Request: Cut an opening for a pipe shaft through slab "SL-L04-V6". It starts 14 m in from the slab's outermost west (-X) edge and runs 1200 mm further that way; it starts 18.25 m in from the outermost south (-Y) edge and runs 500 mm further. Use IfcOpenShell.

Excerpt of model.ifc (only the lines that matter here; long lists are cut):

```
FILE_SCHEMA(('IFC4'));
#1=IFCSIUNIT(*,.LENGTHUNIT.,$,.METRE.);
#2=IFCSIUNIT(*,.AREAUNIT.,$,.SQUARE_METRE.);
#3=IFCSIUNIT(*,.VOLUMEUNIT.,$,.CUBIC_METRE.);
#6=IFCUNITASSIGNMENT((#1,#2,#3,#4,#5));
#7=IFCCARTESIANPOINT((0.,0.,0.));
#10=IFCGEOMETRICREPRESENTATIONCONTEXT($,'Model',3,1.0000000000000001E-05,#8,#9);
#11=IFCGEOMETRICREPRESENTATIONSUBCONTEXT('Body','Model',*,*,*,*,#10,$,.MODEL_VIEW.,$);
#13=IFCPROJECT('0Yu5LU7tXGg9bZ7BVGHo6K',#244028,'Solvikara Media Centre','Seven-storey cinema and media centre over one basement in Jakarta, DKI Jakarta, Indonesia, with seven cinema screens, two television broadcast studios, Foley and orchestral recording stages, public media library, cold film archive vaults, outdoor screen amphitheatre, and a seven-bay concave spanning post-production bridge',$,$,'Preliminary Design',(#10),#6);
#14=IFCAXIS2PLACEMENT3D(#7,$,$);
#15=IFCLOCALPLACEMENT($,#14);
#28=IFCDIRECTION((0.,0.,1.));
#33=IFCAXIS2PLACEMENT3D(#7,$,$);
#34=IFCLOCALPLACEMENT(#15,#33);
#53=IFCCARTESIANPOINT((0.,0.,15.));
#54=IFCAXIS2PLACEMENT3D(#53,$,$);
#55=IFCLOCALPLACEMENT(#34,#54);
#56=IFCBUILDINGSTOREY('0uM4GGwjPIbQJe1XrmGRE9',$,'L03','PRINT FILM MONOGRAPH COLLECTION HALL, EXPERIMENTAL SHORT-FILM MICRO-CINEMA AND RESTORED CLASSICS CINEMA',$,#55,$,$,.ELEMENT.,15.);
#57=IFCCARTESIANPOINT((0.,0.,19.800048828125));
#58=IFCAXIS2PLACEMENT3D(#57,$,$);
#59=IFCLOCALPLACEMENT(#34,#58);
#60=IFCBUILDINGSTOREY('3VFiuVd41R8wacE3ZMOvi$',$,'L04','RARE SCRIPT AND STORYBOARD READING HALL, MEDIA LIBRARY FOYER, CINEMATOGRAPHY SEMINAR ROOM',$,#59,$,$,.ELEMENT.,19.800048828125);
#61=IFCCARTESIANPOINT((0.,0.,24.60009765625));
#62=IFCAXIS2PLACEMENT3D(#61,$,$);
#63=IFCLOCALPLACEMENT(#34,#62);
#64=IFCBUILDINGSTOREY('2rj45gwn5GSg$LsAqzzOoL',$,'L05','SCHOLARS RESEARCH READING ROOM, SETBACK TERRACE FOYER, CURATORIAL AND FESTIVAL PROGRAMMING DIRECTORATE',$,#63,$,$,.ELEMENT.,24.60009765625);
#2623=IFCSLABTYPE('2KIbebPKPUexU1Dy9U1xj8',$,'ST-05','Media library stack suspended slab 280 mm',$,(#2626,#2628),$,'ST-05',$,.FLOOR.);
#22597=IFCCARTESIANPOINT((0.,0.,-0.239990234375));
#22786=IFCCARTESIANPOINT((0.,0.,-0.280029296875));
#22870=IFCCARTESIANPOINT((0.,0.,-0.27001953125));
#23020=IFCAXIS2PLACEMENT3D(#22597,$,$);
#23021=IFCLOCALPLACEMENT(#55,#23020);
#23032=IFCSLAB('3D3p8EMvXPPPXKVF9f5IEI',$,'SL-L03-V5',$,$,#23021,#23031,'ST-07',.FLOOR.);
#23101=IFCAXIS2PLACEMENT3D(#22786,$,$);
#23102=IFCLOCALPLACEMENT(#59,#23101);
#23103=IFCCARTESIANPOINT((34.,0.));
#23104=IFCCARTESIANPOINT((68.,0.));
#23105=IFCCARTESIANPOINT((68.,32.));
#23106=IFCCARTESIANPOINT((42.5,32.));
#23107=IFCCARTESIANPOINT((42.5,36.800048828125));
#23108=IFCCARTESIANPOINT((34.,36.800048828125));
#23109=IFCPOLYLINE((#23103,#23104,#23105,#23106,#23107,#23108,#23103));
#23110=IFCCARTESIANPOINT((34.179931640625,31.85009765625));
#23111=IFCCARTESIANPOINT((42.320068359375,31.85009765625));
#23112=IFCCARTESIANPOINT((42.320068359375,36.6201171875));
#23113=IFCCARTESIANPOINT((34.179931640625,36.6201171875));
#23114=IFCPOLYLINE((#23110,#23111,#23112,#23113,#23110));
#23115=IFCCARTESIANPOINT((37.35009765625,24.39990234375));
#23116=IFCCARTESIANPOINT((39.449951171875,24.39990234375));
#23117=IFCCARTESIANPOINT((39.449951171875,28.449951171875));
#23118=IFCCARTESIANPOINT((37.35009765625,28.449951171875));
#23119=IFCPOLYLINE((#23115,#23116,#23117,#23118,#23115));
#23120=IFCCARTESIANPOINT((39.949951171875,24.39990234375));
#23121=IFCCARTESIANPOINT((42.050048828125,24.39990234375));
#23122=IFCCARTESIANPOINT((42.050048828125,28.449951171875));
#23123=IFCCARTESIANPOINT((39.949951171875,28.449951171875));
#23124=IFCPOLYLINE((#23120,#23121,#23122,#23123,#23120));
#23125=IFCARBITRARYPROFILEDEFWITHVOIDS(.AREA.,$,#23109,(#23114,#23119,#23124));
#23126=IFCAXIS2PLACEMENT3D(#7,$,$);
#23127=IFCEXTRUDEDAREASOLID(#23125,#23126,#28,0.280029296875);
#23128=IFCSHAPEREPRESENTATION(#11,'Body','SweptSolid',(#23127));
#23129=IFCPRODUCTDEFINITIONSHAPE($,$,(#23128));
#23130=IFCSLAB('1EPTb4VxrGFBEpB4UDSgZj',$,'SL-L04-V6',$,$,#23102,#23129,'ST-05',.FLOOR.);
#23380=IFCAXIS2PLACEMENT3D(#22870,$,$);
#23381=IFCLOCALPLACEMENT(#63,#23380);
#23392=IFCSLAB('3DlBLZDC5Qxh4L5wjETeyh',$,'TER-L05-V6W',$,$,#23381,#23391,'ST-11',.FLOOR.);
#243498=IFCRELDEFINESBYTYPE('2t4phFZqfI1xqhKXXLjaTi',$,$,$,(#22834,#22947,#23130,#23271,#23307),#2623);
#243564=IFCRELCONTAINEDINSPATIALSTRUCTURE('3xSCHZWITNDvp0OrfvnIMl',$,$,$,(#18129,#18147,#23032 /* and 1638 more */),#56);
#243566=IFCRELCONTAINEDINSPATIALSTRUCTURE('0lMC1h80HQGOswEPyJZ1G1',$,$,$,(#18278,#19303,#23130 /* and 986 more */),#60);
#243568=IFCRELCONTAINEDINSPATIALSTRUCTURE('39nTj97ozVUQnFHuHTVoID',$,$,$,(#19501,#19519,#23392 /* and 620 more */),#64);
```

```python
import numpy as np
import ifcopenshell
import ifcopenshell.api.feature
import ifcopenshell.api.geometry
import ifcopenshell.api.root
import ifcopenshell.geom
import ifcopenshell.util.placement
import ifcopenshell.util.representation
import ifcopenshell.util.shape
import ifcopenshell.util.unit

model = ifcopenshell.open("model.ifc")
unit_scale = ifcopenshell.util.unit.calculate_unit_scale(model)
settings = ifcopenshell.geom.settings()


def volume(element):
    """Net volume in cubic metres, openings subtracted."""
    shape = ifcopenshell.geom.create_shape(settings, element)
    return ifcopenshell.util.shape.get_volume(shape.geometry)


slab = model.by_id(23130)
before = volume(slab)

# Extent in the slab's own axes, in metres. The edges named are its -X and -Y sides.
slab_shape = ifcopenshell.geom.create_shape(settings, slab)
vertices = ifcopenshell.util.shape.get_vertices(slab_shape.geometry)
x_min, y_min, bottom = vertices.min(axis=0)
top = vertices[:, 2].max()

opening = ifcopenshell.api.root.create_entity(model, ifc_class="IfcOpeningElement", name="Pipe shaft opening", predefined_type="OPENING")
context = ifcopenshell.util.representation.get_context(model, "Model", "Body", "MODEL_VIEW")
width, depth = 1.2, 0.5
outline = [(0.0, 0.0), (width, 0.0), (width, depth), (0.0, depth), (0.0, 0.0)]
# Overshoot both faces by 50 mm so the cut is clean.
shape = ifcopenshell.api.geometry.add_slab_representation(
    model, context=context, depth=top - bottom + 0.1, polyline=outline
)
ifcopenshell.api.geometry.assign_representation(model, product=opening, representation=shape)

matrix = ifcopenshell.util.placement.get_local_placement(slab.ObjectPlacement)
matrix[:, 3] = matrix @ np.append(np.array([x_min + 14, y_min + 18.25, bottom - 0.05]) / unit_scale, 1.0)
ifcopenshell.api.geometry.edit_object_placement(model, product=opening, matrix=matrix, is_si=False)
ifcopenshell.api.feature.add_feature(model, feature=opening, element=slab)

after = volume(slab)

print(f"slab volume {before:.3f} -> {after:.3f} m3")

model.write("model_v2.ifc")
```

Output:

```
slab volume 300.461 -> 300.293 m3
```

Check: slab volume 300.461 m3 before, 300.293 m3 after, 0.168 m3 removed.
